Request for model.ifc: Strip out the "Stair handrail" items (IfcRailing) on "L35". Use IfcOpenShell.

First a look at what the model holds.

```python
import ifcopenshell
import ifcopenshell.util.element

model = ifcopenshell.open("model.ifc")
print(model.schema)
storey = next(s for s in model.by_type("IfcBuildingStorey") if s.Name == "L35")
railings = [e for e in ifcopenshell.util.element.get_decomposition(storey) if e.is_a("IfcRailing")]
seen = {}
for e in railings:
    element_type = ifcopenshell.util.element.get_type(e)
    name = element_type.Name if element_type not in (None, e) else None
    seen[name] = seen.get(name, 0) + 1
for name, count in sorted(seen.items(), key=str):
    print(count, "x", name)
```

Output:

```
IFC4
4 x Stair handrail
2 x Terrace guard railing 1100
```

```python
import ifcopenshell
import ifcopenshell.api.root
import ifcopenshell.util.element

model = ifcopenshell.open("model.ifc")

storey = next(s for s in model.by_type("IfcBuildingStorey") if s.Name == "L35")
railings = [e for e in ifcopenshell.util.element.get_decomposition(storey) if e.is_a("IfcRailing")]
targets = [e for e in railings if (t := ifcopenshell.util.element.get_type(e)) not in (None, e) and t.Name == "Stair handrail"]

for e in targets:
    ifcopenshell.api.root.remove_product(model, product=e)
print(len(targets), "removed")

model.write("model_v2.ifc")
```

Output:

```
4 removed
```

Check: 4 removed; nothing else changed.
